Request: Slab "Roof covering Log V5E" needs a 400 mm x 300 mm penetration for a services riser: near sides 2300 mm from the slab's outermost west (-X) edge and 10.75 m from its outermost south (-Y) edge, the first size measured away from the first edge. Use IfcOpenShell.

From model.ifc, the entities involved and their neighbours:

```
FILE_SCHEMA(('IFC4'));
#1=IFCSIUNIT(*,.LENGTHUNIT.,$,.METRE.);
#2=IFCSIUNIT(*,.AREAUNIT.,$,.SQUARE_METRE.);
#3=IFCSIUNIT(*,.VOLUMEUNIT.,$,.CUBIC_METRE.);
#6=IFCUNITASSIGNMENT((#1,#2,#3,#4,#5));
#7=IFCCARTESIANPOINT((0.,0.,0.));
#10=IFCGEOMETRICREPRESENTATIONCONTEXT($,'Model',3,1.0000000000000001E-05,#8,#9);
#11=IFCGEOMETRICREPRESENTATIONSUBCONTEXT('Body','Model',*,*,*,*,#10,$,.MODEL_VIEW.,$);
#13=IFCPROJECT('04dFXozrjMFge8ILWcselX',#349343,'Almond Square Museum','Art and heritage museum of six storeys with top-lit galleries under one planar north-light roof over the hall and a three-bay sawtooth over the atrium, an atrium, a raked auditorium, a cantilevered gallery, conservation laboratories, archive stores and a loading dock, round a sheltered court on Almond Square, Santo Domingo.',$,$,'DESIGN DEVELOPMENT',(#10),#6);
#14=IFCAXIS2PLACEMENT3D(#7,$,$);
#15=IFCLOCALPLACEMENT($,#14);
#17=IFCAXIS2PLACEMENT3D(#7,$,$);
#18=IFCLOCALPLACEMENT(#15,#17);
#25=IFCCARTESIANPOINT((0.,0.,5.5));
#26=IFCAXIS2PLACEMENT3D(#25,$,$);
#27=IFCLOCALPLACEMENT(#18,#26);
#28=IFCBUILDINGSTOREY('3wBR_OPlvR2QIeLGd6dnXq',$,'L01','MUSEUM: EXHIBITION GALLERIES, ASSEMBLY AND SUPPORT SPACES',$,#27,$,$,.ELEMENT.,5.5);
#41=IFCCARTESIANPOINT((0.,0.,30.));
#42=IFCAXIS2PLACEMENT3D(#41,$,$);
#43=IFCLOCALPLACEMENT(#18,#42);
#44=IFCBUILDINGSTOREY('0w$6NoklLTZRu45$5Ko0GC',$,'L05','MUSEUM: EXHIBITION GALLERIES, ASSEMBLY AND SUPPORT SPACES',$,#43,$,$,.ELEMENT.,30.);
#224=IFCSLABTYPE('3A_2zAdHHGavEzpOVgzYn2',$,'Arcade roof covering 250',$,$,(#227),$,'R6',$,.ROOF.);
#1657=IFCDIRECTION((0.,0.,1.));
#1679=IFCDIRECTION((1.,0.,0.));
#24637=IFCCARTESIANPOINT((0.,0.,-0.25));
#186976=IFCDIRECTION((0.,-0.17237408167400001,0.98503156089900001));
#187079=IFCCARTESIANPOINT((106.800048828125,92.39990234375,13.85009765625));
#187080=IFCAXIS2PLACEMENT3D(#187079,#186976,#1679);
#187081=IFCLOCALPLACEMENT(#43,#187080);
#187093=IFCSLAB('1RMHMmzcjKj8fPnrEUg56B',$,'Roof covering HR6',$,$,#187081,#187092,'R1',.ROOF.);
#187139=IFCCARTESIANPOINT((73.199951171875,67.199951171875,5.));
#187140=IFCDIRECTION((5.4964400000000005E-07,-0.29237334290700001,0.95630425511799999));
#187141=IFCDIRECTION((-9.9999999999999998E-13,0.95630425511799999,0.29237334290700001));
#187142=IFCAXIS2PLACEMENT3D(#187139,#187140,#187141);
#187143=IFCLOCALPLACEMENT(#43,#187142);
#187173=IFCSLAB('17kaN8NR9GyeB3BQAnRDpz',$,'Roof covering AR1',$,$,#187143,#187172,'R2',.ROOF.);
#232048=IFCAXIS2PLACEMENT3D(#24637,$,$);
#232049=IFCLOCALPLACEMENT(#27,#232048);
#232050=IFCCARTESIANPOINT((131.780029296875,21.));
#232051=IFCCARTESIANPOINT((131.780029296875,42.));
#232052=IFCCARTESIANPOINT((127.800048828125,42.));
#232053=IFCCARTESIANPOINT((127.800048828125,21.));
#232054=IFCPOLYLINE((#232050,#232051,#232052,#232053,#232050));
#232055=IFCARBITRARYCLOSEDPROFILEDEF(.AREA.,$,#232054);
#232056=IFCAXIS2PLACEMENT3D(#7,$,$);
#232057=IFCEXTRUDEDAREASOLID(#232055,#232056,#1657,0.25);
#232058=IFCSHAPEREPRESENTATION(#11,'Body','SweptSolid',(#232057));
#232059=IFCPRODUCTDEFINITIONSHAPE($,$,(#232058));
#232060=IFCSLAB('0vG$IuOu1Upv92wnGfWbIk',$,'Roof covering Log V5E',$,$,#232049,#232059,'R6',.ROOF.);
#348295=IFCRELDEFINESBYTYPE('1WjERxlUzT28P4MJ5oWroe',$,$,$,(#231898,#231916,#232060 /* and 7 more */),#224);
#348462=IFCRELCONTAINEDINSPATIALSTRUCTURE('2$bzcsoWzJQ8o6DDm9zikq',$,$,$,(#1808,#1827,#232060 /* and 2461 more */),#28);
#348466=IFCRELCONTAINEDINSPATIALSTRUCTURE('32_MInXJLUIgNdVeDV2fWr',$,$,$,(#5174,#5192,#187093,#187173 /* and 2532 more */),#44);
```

```python
import numpy as np
import ifcopenshell
import ifcopenshell.api.feature
import ifcopenshell.api.geometry
import ifcopenshell.api.root
import ifcopenshell.geom
import ifcopenshell.util.placement
import ifcopenshell.util.representation
import ifcopenshell.util.shape
import ifcopenshell.util.unit

model = ifcopenshell.open("model.ifc")
unit_scale = ifcopenshell.util.unit.calculate_unit_scale(model)
settings = ifcopenshell.geom.settings()


def volume(element):
    """Net volume in cubic metres, openings subtracted."""
    shape = ifcopenshell.geom.create_shape(settings, element)
    return ifcopenshell.util.shape.get_volume(shape.geometry)


slab = model.by_guid("0vG$IuOu1Upv92wnGfWbIk")
before = volume(slab)

# Extent in the slab's own axes, in metres. The edges named are its -X and -Y sides.
slab_shape = ifcopenshell.geom.create_shape(settings, slab)
vertices = ifcopenshell.util.shape.get_vertices(slab_shape.geometry)
x_min, y_min, bottom = vertices.min(axis=0)
top = vertices[:, 2].max()

opening = ifcopenshell.api.root.create_entity(model, ifc_class="IfcOpeningElement", name="Services riser opening", predefined_type="OPENING")
context = ifcopenshell.util.representation.get_context(model, "Model", "Body", "MODEL_VIEW")
width, depth = 0.4, 0.3
outline = [(0.0, 0.0), (width, 0.0), (width, depth), (0.0, depth), (0.0, 0.0)]
# Overshoot both faces by 50 mm so the cut is clean.
shape = ifcopenshell.api.geometry.add_slab_representation(
    model, context=context, depth=top - bottom + 0.1, polyline=outline
)
ifcopenshell.api.geometry.assign_representation(model, product=opening, representation=shape)

matrix = ifcopenshell.util.placement.get_local_placement(slab.ObjectPlacement)
matrix[:, 3] = matrix @ np.append(np.array([x_min + 2.3, y_min + 10.75, bottom - 0.05]) / unit_scale, 1.0)
ifcopenshell.api.geometry.edit_object_placement(model, product=opening, matrix=matrix, is_si=False)
ifcopenshell.api.feature.add_feature(model, feature=opening, element=slab)

after = volume(slab)

print(f"slab volume {before:.3f} -> {after:.3f} m3")

model.write("model-out.ifc")
```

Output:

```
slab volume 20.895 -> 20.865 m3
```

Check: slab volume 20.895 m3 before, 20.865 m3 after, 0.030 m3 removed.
